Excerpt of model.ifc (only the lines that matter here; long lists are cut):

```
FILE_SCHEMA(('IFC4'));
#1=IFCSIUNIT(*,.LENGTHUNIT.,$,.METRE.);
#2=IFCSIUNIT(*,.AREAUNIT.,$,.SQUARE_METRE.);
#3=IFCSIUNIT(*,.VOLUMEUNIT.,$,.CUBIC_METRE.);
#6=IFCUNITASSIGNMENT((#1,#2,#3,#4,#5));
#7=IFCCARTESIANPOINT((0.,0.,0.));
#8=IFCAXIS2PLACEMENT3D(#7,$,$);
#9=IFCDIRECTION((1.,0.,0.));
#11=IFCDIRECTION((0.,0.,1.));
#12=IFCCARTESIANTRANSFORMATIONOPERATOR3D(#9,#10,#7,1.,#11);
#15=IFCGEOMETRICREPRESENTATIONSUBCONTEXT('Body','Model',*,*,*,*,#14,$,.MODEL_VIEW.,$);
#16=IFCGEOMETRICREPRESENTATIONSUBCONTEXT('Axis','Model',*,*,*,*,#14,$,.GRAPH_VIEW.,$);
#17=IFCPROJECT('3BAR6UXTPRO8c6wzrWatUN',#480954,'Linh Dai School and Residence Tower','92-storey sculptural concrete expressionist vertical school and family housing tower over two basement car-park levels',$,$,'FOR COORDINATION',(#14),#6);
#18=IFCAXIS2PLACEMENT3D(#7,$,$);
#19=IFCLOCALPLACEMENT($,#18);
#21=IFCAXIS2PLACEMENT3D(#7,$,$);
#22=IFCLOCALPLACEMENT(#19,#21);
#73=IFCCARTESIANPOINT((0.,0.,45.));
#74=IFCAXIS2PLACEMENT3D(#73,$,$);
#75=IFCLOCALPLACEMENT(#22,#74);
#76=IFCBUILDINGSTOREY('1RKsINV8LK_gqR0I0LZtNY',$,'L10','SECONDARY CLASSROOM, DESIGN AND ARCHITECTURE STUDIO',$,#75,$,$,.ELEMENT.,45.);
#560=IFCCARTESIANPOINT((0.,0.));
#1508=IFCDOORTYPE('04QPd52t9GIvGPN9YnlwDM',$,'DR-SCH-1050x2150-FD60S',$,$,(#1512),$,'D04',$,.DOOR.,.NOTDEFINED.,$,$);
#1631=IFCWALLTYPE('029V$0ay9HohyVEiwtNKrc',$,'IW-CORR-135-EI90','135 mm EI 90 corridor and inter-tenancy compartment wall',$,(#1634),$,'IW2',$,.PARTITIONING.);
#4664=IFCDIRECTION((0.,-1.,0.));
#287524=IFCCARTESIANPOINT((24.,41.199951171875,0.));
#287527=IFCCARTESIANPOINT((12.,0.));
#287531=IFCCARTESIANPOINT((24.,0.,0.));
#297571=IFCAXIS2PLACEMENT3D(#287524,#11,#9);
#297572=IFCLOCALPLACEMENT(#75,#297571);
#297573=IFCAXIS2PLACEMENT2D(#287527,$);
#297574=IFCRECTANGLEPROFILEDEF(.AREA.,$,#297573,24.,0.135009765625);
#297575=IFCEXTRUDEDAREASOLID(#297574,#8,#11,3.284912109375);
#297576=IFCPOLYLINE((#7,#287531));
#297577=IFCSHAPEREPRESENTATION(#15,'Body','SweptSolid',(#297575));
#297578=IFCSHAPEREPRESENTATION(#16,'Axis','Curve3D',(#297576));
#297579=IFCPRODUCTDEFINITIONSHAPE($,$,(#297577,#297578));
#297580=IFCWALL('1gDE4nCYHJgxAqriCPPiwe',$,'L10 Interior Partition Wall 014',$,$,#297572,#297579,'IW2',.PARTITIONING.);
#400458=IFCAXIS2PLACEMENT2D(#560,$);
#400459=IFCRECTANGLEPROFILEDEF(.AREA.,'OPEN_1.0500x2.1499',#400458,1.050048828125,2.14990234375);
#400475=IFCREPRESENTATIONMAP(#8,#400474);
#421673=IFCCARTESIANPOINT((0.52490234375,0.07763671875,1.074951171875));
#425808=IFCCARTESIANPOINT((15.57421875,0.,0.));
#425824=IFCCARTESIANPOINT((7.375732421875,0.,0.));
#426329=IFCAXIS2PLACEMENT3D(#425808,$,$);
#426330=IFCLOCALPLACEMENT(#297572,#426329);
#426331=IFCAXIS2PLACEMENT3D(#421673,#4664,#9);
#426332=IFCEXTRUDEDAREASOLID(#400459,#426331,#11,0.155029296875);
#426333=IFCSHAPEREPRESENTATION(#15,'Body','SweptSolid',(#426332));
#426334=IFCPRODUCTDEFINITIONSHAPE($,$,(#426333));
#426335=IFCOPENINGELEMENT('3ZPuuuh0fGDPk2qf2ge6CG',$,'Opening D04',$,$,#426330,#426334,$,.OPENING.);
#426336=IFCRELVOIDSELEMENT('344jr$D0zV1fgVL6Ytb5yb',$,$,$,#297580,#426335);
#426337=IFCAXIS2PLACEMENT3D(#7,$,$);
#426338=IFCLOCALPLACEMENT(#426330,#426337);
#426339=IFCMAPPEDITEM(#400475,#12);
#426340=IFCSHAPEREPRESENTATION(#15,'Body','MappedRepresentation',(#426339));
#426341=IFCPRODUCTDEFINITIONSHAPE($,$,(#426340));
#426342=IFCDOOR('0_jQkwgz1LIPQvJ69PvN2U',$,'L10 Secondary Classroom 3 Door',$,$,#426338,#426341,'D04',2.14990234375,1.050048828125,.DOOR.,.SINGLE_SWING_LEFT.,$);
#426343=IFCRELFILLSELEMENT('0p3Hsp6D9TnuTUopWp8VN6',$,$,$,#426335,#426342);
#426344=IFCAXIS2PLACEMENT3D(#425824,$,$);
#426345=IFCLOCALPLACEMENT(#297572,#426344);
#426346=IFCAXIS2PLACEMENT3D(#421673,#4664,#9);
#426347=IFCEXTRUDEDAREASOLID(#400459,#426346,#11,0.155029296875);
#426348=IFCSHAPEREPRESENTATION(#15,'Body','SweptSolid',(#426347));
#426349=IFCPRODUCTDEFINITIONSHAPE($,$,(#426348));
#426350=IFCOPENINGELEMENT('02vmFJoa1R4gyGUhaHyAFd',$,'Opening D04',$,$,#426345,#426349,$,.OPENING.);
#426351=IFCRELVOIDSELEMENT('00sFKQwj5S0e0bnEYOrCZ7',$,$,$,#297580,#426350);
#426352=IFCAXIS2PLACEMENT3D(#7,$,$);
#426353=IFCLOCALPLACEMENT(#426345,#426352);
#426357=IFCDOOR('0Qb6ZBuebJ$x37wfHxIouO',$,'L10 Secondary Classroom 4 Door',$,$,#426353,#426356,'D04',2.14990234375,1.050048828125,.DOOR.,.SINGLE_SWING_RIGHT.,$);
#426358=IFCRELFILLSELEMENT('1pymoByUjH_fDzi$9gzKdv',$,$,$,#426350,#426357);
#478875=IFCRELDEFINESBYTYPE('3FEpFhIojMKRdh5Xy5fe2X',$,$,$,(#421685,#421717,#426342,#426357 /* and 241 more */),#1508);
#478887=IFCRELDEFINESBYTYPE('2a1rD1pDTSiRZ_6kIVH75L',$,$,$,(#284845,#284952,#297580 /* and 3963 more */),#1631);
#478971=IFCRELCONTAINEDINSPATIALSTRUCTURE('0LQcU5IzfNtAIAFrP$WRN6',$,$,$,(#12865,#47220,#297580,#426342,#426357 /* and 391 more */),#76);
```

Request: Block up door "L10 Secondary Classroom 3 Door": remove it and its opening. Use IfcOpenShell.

```python
import ifcopenshell
import ifcopenshell.api.feature
import ifcopenshell.api.root
import ifcopenshell.geom
import ifcopenshell.util.shape

model = ifcopenshell.open("model.ifc")
settings = ifcopenshell.geom.settings()


def volume(element):
    """Net volume in cubic metres, openings subtracted."""
    shape = ifcopenshell.geom.create_shape(settings, element)
    return ifcopenshell.util.shape.get_volume(shape.geometry)


door = model.by_id(426342)
opening = door.FillsVoids[0].RelatingOpeningElement
wall = opening.VoidsElements[0].RelatingBuildingElement
before = volume(wall)

ifcopenshell.api.root.remove_product(model, product=door)
ifcopenshell.api.feature.remove_feature(model, feature=opening)

after = volume(wall)

print(f"wall volume {before:.3f} -> {after:.3f} m3")

model.write("model-out.ifc")
```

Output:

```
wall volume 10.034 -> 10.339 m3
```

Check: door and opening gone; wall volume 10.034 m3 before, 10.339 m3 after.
